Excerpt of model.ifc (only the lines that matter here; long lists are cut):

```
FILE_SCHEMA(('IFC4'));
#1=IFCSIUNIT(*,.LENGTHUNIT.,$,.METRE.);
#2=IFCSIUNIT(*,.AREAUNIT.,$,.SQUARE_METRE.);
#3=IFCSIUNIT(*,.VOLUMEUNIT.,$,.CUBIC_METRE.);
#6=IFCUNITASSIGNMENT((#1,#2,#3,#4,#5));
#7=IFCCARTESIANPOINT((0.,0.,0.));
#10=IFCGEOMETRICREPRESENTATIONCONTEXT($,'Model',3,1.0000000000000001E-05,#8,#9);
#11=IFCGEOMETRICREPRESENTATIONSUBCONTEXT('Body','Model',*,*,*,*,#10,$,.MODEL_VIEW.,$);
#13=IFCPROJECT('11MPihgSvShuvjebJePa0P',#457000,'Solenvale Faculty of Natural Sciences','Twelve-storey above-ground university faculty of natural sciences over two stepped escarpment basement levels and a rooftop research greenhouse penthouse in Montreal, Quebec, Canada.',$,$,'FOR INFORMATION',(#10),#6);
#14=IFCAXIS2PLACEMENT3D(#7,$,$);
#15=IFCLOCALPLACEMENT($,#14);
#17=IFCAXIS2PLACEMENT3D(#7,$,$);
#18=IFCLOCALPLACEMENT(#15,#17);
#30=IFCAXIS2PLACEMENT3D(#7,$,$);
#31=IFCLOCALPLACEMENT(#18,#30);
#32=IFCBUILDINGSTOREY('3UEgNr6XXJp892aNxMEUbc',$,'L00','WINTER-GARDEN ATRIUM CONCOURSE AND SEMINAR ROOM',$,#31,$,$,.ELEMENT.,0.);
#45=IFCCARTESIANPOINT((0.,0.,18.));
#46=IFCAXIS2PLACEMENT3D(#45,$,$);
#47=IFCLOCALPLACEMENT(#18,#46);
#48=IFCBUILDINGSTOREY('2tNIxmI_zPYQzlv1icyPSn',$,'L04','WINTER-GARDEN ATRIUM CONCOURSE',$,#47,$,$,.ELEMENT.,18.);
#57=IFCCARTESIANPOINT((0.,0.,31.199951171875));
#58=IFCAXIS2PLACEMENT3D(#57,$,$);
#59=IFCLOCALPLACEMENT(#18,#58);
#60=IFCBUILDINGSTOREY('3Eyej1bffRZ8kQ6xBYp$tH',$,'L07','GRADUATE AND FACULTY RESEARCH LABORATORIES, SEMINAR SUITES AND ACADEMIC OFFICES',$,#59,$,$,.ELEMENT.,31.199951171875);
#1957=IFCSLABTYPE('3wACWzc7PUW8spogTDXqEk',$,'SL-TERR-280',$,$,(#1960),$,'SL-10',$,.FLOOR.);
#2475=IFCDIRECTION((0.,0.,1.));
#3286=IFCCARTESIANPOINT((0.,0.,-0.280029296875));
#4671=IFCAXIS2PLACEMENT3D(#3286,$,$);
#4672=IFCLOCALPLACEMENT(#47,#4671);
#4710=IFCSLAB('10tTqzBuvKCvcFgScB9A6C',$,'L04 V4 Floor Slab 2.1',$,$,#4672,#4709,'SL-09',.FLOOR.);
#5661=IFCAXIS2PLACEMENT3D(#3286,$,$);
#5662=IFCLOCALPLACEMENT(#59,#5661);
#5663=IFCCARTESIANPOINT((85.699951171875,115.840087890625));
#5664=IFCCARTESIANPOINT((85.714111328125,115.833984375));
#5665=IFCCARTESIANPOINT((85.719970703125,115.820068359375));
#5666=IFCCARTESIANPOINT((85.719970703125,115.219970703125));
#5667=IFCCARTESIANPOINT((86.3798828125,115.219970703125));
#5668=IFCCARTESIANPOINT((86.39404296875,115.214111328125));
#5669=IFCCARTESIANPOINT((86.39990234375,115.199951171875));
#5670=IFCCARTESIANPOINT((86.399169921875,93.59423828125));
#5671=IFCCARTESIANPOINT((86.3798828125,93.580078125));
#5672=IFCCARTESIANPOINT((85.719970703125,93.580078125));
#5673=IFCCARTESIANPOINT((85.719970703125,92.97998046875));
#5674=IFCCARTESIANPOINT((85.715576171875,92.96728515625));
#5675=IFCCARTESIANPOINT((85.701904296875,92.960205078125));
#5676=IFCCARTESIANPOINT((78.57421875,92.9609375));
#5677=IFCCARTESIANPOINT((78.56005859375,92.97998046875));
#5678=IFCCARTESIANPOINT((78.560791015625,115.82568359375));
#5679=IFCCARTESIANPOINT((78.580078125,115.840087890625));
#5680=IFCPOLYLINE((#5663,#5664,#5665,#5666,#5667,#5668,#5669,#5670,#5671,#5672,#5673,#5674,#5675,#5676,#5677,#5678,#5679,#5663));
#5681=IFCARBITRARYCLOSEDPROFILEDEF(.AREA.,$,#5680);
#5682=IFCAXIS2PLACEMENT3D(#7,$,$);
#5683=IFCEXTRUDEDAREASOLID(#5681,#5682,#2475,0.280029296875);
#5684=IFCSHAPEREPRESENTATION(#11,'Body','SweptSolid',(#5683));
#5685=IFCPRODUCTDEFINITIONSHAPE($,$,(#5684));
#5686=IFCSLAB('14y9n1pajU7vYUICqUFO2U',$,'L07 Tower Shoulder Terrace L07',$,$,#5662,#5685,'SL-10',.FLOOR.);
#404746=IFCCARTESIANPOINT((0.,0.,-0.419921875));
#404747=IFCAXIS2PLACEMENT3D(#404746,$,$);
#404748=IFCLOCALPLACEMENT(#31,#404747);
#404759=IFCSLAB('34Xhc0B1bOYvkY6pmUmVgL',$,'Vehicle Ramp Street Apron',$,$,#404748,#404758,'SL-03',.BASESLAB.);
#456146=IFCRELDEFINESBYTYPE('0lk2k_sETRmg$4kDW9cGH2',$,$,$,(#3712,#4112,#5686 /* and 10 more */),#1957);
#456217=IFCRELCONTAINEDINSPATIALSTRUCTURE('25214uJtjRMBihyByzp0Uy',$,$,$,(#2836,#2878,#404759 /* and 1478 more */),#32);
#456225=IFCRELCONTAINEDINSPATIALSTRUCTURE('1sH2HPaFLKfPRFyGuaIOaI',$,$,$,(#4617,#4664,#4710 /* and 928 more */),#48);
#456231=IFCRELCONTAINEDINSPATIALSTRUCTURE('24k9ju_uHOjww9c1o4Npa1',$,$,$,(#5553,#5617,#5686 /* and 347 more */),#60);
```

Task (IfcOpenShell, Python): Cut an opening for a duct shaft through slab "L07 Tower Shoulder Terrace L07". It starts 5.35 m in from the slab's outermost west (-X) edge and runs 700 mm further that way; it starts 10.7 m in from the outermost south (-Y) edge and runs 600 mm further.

```python
import numpy as np
import ifcopenshell
import ifcopenshell.api.feature
import ifcopenshell.api.geometry
import ifcopenshell.api.root
import ifcopenshell.geom
import ifcopenshell.util.placement
import ifcopenshell.util.representation
import ifcopenshell.util.shape
import ifcopenshell.util.unit

model = ifcopenshell.open("model.ifc")
unit_scale = ifcopenshell.util.unit.calculate_unit_scale(model)
settings = ifcopenshell.geom.settings()


def volume(element):
    """Net volume in cubic metres, openings subtracted."""
    shape = ifcopenshell.geom.create_shape(settings, element)
    return ifcopenshell.util.shape.get_volume(shape.geometry)


slab = model.by_guid("14y9n1pajU7vYUICqUFO2U")
before = volume(slab)

# Extent in the slab's own axes, in metres. The edges named are its -X and -Y sides.
slab_shape = ifcopenshell.geom.create_shape(settings, slab)
vertices = ifcopenshell.util.shape.get_vertices(slab_shape.geometry)
x_min, y_min, bottom = vertices.min(axis=0)
top = vertices[:, 2].max()

opening = ifcopenshell.api.root.create_entity(model, ifc_class="IfcOpeningElement", name="Duct shaft opening", predefined_type="OPENING")
context = ifcopenshell.util.representation.get_context(model, "Model", "Body", "MODEL_VIEW")
width, depth = 0.7, 0.6
outline = [(0.0, 0.0), (width, 0.0), (width, depth), (0.0, depth), (0.0, 0.0)]
# Overshoot both faces by 50 mm so the cut is clean.
shape = ifcopenshell.api.geometry.add_slab_representation(
    model, context=context, depth=top - bottom + 0.1, polyline=outline
)
ifcopenshell.api.geometry.assign_representation(model, product=opening, representation=shape)

matrix = ifcopenshell.util.placement.get_local_placement(slab.ObjectPlacement)
matrix[:, 3] = matrix @ np.append(np.array([x_min + 5.35, y_min + 10.7, bottom - 0.05]) / unit_scale, 1.0)
ifcopenshell.api.geometry.edit_object_placement(model, product=opening, matrix=matrix, is_si=False)
ifcopenshell.api.feature.add_feature(model, feature=opening, element=slab)

after = volume(slab)

print(f"slab volume {before:.3f} -> {after:.3f} m3")

model.write("model_updated.ifc")
```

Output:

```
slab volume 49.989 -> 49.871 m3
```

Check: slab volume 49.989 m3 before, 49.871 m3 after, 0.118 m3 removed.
